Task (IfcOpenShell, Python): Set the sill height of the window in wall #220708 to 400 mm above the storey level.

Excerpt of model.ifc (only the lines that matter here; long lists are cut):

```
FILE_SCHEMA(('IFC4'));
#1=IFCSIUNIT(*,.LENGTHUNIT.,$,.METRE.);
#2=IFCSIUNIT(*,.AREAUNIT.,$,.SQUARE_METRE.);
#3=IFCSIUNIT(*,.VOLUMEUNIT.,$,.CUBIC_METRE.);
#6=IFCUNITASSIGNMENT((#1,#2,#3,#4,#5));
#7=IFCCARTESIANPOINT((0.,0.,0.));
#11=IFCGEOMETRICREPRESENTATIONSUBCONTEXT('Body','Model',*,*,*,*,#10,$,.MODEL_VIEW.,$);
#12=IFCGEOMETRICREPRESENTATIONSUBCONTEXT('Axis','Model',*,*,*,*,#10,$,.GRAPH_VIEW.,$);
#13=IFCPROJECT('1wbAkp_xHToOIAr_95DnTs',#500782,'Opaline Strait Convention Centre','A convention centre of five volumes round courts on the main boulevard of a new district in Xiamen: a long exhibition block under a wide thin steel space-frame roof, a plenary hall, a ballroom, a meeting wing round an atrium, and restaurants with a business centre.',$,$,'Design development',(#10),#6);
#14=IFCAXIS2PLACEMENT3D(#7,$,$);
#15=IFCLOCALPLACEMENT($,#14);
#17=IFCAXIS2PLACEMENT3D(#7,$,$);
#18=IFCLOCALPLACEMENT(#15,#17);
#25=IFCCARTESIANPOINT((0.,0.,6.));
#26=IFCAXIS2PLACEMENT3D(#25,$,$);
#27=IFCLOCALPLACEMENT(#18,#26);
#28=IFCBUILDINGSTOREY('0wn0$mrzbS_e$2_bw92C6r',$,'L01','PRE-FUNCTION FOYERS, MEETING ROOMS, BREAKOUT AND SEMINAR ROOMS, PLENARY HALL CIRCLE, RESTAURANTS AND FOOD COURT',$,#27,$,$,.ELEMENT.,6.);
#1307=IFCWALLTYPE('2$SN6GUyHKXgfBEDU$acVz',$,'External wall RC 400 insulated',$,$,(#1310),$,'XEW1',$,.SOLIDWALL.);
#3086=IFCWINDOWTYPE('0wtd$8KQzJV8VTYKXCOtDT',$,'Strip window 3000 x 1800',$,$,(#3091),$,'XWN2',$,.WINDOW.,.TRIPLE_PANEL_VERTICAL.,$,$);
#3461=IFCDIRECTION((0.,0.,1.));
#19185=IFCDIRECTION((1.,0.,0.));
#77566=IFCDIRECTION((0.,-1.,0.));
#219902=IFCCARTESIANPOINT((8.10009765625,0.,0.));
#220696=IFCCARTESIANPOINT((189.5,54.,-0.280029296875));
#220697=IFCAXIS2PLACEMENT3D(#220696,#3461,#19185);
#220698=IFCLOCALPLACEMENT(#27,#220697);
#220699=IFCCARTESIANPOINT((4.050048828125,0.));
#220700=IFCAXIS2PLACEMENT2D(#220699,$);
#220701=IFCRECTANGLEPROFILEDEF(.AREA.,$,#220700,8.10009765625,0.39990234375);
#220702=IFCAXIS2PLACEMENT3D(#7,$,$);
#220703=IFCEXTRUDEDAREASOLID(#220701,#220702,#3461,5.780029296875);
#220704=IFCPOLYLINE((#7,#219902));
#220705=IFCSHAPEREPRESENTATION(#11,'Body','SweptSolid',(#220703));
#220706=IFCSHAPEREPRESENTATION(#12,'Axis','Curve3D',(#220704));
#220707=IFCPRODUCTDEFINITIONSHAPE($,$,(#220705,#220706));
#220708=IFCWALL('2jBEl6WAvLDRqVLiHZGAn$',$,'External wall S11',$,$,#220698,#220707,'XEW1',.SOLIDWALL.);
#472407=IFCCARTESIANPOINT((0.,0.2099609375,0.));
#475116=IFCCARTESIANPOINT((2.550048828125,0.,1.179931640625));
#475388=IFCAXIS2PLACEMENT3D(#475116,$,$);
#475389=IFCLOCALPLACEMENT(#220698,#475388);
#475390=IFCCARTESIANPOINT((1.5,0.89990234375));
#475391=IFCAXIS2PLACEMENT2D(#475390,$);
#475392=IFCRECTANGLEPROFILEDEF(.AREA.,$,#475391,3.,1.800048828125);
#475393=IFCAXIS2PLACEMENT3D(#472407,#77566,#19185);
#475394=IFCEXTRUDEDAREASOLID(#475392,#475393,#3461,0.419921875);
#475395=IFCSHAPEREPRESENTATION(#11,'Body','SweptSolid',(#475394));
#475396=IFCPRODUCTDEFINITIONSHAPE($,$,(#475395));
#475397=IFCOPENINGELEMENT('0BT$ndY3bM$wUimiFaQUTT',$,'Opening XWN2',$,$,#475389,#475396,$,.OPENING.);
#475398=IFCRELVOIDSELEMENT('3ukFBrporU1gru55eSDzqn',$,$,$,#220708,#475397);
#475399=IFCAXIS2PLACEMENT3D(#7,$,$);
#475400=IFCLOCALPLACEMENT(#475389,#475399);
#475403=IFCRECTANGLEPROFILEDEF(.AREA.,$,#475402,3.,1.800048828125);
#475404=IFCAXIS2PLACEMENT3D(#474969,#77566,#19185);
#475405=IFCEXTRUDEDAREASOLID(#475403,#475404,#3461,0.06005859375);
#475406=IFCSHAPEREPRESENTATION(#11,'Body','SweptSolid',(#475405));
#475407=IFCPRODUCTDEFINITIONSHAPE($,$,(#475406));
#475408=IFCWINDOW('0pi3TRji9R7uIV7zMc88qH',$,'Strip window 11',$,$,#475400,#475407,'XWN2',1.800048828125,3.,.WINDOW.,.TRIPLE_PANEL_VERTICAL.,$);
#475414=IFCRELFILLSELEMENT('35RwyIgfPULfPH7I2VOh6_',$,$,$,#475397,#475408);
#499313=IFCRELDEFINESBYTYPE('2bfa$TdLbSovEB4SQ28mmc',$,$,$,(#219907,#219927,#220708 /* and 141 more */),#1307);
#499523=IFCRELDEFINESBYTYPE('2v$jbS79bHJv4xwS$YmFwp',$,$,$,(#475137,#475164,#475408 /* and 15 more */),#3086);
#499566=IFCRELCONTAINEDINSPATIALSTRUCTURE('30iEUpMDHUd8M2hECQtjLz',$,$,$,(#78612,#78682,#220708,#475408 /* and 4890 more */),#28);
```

```python
import numpy as np
import ifcopenshell
import ifcopenshell.api.geometry
import ifcopenshell.geom
import ifcopenshell.util.element
import ifcopenshell.util.placement
import ifcopenshell.util.shape
import ifcopenshell.util.unit

model = ifcopenshell.open("model.ifc")
unit_scale = ifcopenshell.util.unit.calculate_unit_scale(model)

window = model.by_guid("0pi3TRji9R7uIV7zMc88qH")
opening = window.FillsVoids[0].RelatingOpeningElement
storey = ifcopenshell.util.element.get_container(window, ifc_class="IfcBuildingStorey")
level = ifcopenshell.util.placement.get_local_placement(storey.ObjectPlacement)[2, 3]

# The opening's origin need not be at the sill, so measure its lowest point.
shape = ifcopenshell.geom.create_shape(ifcopenshell.geom.settings(), opening)
bottom = ifcopenshell.util.shape.get_shape_bottom_elevation(shape, shape.geometry) / unit_scale
dz = level + 0.4 - bottom

shift = np.array([0.0, 0.0, dz])
# The window is placed relative to its opening, so it follows when the opening moves.
matrix = ifcopenshell.util.placement.get_local_placement(opening.ObjectPlacement)
matrix[:3, 3] += shift
ifcopenshell.api.geometry.edit_object_placement(
    model, product=opening, matrix=matrix, is_si=False, should_transform_children=True
)

print(f"moved by {dz * unit_scale:+.3f} m")

model.write("model-out.ifc")
```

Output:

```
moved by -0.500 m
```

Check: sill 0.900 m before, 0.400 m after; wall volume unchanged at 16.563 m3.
